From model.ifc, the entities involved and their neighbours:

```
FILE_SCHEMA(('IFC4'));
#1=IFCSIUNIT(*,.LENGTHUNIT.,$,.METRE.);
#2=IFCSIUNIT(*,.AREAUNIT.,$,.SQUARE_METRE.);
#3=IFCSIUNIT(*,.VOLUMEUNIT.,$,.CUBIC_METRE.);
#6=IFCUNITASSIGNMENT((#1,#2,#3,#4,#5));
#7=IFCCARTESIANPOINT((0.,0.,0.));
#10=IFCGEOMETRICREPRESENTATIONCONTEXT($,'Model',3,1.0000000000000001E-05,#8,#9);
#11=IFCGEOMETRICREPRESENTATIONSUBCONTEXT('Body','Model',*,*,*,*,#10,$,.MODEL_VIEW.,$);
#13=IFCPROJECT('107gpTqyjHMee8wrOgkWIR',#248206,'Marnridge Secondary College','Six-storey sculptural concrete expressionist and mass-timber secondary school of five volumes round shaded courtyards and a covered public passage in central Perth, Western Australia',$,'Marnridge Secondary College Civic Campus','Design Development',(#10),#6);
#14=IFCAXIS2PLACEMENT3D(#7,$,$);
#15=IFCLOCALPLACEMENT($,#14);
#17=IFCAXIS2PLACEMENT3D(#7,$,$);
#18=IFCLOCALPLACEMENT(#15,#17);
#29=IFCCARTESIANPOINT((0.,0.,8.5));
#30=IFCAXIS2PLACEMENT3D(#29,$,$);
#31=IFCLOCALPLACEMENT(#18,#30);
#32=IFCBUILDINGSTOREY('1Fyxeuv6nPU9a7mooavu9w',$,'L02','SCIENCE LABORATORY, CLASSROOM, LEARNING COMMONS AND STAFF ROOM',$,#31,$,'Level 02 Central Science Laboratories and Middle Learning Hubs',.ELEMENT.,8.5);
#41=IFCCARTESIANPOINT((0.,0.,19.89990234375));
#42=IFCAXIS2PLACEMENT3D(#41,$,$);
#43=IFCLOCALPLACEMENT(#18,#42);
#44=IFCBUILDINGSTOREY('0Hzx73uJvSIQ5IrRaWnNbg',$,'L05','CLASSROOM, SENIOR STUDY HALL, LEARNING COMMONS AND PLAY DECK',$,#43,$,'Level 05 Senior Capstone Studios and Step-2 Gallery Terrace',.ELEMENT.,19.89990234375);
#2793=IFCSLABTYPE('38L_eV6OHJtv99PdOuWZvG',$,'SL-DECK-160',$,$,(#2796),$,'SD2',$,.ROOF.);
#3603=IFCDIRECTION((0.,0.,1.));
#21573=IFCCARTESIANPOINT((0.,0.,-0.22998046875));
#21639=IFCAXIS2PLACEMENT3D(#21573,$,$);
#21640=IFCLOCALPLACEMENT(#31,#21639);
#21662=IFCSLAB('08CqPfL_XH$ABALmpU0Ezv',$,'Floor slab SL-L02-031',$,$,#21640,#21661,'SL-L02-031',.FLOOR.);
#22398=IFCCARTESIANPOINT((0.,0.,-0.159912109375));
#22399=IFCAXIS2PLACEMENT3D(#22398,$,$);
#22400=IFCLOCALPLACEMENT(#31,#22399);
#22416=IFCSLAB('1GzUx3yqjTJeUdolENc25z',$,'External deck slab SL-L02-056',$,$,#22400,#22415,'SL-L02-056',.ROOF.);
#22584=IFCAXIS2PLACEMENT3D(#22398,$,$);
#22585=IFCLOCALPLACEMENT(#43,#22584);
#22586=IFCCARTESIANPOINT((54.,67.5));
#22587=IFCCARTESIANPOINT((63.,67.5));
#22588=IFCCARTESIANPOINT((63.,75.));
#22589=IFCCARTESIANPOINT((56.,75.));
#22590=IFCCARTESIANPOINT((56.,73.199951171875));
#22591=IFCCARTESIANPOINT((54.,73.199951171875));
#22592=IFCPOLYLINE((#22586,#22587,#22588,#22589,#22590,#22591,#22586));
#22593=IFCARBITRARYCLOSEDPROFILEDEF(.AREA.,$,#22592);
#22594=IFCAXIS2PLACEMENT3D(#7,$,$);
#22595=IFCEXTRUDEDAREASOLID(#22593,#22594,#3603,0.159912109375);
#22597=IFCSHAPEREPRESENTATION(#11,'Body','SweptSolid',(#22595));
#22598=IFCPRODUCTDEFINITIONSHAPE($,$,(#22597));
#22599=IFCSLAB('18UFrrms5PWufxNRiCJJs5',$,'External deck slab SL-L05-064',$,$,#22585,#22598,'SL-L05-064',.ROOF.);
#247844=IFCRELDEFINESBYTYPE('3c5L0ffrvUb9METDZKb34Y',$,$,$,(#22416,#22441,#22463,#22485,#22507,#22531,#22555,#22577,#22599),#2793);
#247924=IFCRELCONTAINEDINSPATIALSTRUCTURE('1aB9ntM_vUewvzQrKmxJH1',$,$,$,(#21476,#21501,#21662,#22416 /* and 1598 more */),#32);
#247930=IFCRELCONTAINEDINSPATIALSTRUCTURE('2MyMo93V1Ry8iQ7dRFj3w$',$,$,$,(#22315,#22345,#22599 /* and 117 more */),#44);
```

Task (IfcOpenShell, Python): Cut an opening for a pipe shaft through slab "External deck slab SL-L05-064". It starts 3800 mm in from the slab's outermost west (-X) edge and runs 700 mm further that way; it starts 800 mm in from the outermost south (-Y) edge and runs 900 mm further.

```python
import numpy as np
import ifcopenshell
import ifcopenshell.api.feature
import ifcopenshell.api.geometry
import ifcopenshell.api.root
import ifcopenshell.geom
import ifcopenshell.util.placement
import ifcopenshell.util.representation
import ifcopenshell.util.shape
import ifcopenshell.util.unit

model = ifcopenshell.open("model.ifc")
unit_scale = ifcopenshell.util.unit.calculate_unit_scale(model)
settings = ifcopenshell.geom.settings()


def volume(element):
    """Net volume in cubic metres, openings subtracted."""
    shape = ifcopenshell.geom.create_shape(settings, element)
    return ifcopenshell.util.shape.get_volume(shape.geometry)


slab = model.by_guid("18UFrrms5PWufxNRiCJJs5")
before = volume(slab)

# Extent in the slab's own axes, in metres. The edges named are its -X and -Y sides.
slab_shape = ifcopenshell.geom.create_shape(settings, slab)
vertices = ifcopenshell.util.shape.get_vertices(slab_shape.geometry)
x_min, y_min, bottom = vertices.min(axis=0)
top = vertices[:, 2].max()

opening = ifcopenshell.api.root.create_entity(model, ifc_class="IfcOpeningElement", name="Pipe shaft opening", predefined_type="OPENING")
context = ifcopenshell.util.representation.get_context(model, "Model", "Body", "MODEL_VIEW")
width, depth = 0.7, 0.9
outline = [(0.0, 0.0), (width, 0.0), (width, depth), (0.0, depth), (0.0, 0.0)]
# Overshoot both faces by 50 mm so the cut is clean.
shape = ifcopenshell.api.geometry.add_slab_representation(
    model, context=context, depth=top - bottom + 0.1, polyline=outline
)
ifcopenshell.api.geometry.assign_representation(model, product=opening, representation=shape)

matrix = ifcopenshell.util.placement.get_local_placement(slab.ObjectPlacement)
matrix[:, 3] = matrix @ np.append(np.array([x_min + 3.8, y_min + 0.8, bottom - 0.05]) / unit_scale, 1.0)
ifcopenshell.api.geometry.edit_object_placement(model, product=opening, matrix=matrix, is_si=False)
ifcopenshell.api.feature.add_feature(model, feature=opening, element=slab)

after = volume(slab)

print(f"slab volume {before:.3f} -> {after:.3f} m3")

model.write("model-out.ifc")
```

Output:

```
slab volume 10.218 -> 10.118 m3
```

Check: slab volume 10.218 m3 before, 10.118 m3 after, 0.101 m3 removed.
